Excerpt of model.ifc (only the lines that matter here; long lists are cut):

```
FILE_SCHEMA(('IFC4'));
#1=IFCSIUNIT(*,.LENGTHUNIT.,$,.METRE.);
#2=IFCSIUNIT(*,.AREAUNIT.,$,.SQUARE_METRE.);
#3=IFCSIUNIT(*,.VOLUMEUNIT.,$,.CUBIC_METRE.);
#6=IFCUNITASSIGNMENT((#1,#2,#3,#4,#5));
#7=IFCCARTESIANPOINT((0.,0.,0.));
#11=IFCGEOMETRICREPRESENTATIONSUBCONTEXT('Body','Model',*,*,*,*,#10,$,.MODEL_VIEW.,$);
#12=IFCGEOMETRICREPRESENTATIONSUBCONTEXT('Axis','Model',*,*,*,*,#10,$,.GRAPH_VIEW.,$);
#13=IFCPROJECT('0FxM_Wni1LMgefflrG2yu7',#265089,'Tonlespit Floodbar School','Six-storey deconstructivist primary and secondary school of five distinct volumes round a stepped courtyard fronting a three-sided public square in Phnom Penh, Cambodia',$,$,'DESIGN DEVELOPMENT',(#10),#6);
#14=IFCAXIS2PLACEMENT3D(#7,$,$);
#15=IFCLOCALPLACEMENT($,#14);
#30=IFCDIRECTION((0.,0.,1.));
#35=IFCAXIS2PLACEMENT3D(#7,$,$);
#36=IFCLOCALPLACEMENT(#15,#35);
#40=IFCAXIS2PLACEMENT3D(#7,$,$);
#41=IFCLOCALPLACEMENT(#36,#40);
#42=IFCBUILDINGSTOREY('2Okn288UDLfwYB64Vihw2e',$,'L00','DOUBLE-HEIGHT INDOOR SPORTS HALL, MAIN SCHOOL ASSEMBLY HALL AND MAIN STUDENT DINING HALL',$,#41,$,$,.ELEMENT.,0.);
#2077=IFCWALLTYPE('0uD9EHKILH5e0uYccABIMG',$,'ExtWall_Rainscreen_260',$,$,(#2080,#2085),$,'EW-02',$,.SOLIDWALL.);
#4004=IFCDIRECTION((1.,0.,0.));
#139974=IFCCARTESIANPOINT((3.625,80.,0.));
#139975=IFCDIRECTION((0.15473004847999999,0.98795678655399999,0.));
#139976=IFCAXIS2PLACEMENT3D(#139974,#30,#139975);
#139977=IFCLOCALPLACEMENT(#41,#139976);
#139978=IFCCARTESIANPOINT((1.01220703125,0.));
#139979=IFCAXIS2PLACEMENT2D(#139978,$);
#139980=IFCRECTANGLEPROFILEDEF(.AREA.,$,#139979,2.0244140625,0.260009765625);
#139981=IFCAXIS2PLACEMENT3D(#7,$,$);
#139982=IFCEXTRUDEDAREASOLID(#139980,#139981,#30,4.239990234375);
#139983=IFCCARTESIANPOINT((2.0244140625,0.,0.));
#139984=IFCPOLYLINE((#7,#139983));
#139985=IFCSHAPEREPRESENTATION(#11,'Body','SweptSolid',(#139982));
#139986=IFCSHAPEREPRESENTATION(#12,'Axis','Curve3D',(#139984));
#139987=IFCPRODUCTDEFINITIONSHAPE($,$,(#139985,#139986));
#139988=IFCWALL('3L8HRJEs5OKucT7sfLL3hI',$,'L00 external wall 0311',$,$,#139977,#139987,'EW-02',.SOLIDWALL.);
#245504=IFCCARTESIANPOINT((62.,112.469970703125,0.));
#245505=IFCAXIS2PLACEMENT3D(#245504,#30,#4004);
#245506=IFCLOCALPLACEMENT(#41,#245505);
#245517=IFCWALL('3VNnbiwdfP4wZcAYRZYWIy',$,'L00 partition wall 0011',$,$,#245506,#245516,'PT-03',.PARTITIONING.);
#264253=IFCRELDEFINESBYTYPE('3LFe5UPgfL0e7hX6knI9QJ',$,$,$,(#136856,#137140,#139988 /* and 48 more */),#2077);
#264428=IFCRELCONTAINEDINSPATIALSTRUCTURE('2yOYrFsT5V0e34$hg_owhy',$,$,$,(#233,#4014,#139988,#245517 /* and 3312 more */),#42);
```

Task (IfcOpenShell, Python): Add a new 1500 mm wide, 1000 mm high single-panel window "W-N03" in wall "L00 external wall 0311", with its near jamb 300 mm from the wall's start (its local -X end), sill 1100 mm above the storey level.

```python
import numpy as np
import ifcopenshell
import ifcopenshell.api.feature
import ifcopenshell.api.geometry
import ifcopenshell.api.root
import ifcopenshell.api.spatial
import ifcopenshell.geom
import ifcopenshell.util.element
import ifcopenshell.util.placement
import ifcopenshell.util.representation
import ifcopenshell.util.shape
import ifcopenshell.util.unit

model = ifcopenshell.open("model.ifc")
unit_scale = ifcopenshell.util.unit.calculate_unit_scale(model)
settings = ifcopenshell.geom.settings()


def volume(element):
    """Net volume in cubic metres, openings subtracted."""
    shape = ifcopenshell.geom.create_shape(settings, element)
    return ifcopenshell.util.shape.get_volume(shape.geometry)


wall = model.by_guid("3L8HRJEs5OKucT7sfLL3hI")
storey = ifcopenshell.util.element.get_container(wall, ifc_class="IfcBuildingStorey")
context = ifcopenshell.util.representation.get_context(model, "Model", "Body", "MODEL_VIEW")
before = volume(wall)

width, height, from_end, sill = 1.5, 1, 0.3, 1.1  # metres

# The wall runs along its own X axis, and the end named is its -X end.
wall_shape = ifcopenshell.geom.create_shape(settings, wall)
x, y, z = ifcopenshell.util.shape.get_vertices(wall_shape.geometry).T
start = x.min() + from_end
face, thickness = float(y.min()), float(y.max() - y.min())
wall_matrix = ifcopenshell.util.placement.get_local_placement(wall.ObjectPlacement)
level = ifcopenshell.util.placement.get_local_placement(storey.ObjectPlacement)[2, 3]


def in_wall(x, y):
    """Placement at x, y metres in the wall's axes, at sill height."""
    matrix = wall_matrix.copy()
    matrix[:, 3] = wall_matrix @ np.array([x / unit_scale, y / unit_scale, 0.0, 1.0])
    matrix[2, 3] = level + sill / unit_scale
    return matrix


# Opening: a box that overshoots both wall faces by 50 mm.
opening = ifcopenshell.api.root.create_entity(model, ifc_class="IfcOpeningElement", predefined_type="OPENING")
box = ifcopenshell.api.geometry.add_wall_representation(
    model, context=context, length=width, height=height, thickness=thickness + 0.1
)
ifcopenshell.api.geometry.assign_representation(model, product=opening, representation=box)
ifcopenshell.api.geometry.edit_object_placement(model, product=opening, matrix=in_wall(start, face - 0.05), is_si=False)
ifcopenshell.api.feature.add_feature(model, feature=opening, element=wall)

window = ifcopenshell.api.root.create_entity(model, ifc_class="IfcWindow", name="W-N03", predefined_type="WINDOW")
window.OverallWidth, window.OverallHeight = width / unit_scale, height / unit_scale
window.PartitioningType = "SINGLE_PANEL"
body = ifcopenshell.api.geometry.add_window_representation(
    model,
    context=context,
    overall_width=window.OverallWidth,
    overall_height=window.OverallHeight,
    partition_type="SINGLE_PANEL",
)
ifcopenshell.api.geometry.assign_representation(model, product=window, representation=body)
ifcopenshell.api.spatial.assign_container(model, products=[window], relating_structure=storey)
ifcopenshell.api.feature.add_filling(model, opening=opening, element=window)

# Centre the window in the wall's thickness.
ifcopenshell.api.geometry.edit_object_placement(model, product=window, matrix=in_wall(start, face), is_si=False)
window_shape = ifcopenshell.geom.create_shape(settings, window)
depth = ifcopenshell.util.shape.get_vertices(window_shape.geometry)[:, 1]
offset = face + thickness / 2 - (depth.min() + depth.max()) / 2
ifcopenshell.api.geometry.edit_object_placement(model, product=window, matrix=in_wall(start, offset), is_si=False)

after = volume(wall)

print(f"wall volume {before:.3f} -> {after:.3f} m3")

model.write("model_updated.ifc")
```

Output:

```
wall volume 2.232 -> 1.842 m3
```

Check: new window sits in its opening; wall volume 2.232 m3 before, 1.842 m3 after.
